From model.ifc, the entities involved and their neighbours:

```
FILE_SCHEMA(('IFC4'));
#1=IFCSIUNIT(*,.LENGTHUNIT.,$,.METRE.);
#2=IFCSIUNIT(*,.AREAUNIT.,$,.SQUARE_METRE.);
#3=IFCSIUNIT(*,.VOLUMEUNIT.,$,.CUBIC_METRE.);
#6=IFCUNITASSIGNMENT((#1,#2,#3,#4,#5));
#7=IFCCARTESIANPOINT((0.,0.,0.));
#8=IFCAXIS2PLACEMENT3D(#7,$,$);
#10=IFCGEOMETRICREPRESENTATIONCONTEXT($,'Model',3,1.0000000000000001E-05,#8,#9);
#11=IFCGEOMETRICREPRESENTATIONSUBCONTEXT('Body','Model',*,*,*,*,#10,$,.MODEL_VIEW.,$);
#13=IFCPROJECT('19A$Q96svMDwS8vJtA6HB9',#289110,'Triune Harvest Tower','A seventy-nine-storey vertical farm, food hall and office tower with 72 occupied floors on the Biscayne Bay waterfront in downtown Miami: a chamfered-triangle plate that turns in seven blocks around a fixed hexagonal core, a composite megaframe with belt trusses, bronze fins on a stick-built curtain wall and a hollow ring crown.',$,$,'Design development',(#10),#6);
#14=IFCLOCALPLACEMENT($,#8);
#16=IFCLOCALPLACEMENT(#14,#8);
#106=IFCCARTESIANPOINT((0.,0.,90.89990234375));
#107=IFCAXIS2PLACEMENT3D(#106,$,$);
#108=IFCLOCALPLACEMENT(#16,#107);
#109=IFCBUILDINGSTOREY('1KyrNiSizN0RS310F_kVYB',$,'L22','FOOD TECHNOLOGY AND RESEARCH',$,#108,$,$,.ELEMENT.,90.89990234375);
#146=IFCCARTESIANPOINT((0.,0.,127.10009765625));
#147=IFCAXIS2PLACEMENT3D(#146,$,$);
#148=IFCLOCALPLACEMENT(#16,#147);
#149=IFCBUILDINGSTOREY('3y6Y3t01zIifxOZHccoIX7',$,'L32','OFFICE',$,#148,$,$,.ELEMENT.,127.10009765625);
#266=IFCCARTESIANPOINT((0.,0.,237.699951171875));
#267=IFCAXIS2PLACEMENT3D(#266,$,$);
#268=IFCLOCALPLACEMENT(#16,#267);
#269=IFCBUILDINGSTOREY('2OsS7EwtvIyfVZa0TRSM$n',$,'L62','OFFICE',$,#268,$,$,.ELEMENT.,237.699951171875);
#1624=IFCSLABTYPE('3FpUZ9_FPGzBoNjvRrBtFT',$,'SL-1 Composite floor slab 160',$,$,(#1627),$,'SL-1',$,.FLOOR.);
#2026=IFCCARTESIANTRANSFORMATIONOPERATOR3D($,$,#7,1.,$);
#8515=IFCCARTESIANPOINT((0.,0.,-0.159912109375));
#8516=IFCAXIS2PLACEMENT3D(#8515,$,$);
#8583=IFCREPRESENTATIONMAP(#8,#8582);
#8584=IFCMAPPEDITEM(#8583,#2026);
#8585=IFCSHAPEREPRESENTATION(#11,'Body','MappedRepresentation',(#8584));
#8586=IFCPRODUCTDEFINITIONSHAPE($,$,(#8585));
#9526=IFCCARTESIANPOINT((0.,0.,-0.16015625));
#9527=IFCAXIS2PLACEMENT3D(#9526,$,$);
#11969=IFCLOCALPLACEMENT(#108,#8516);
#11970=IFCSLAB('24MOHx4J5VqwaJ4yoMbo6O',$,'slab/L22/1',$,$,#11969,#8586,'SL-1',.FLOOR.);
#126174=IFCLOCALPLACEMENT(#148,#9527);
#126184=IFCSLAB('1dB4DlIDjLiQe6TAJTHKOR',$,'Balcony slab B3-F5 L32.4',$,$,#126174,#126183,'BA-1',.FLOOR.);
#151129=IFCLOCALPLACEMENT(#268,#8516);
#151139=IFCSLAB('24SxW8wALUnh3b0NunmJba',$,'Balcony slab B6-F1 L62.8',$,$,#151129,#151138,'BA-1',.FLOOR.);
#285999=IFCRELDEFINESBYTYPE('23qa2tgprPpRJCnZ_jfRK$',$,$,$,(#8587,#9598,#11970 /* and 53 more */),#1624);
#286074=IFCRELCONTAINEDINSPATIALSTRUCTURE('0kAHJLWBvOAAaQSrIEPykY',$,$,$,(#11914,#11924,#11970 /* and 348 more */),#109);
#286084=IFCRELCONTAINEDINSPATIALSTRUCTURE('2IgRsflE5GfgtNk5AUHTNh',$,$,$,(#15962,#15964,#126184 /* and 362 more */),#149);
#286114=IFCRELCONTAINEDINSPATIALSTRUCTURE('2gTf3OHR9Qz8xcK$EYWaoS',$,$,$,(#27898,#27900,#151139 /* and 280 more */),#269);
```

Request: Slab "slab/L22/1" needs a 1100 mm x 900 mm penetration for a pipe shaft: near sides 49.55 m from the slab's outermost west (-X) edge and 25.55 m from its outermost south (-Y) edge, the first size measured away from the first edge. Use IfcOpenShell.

```python
import numpy as np
import ifcopenshell
import ifcopenshell.api.feature
import ifcopenshell.api.geometry
import ifcopenshell.api.root
import ifcopenshell.geom
import ifcopenshell.util.placement
import ifcopenshell.util.representation
import ifcopenshell.util.shape
import ifcopenshell.util.unit

model = ifcopenshell.open("model.ifc")
unit_scale = ifcopenshell.util.unit.calculate_unit_scale(model)
settings = ifcopenshell.geom.settings()


def volume(element):
    """Net volume in cubic metres, openings subtracted."""
    shape = ifcopenshell.geom.create_shape(settings, element)
    return ifcopenshell.util.shape.get_volume(shape.geometry)


slab = model.by_guid("24MOHx4J5VqwaJ4yoMbo6O")
before = volume(slab)

# Extent in the slab's own axes, in metres. The edges named are its -X and -Y sides.
slab_shape = ifcopenshell.geom.create_shape(settings, slab)
vertices = ifcopenshell.util.shape.get_vertices(slab_shape.geometry)
x_min, y_min, bottom = vertices.min(axis=0)
top = vertices[:, 2].max()

opening = ifcopenshell.api.root.create_entity(model, ifc_class="IfcOpeningElement", name="Pipe shaft opening", predefined_type="OPENING")
context = ifcopenshell.util.representation.get_context(model, "Model", "Body", "MODEL_VIEW")
width, depth = 1.1, 0.9
outline = [(0.0, 0.0), (width, 0.0), (width, depth), (0.0, depth), (0.0, 0.0)]
# Overshoot both faces by 50 mm so the cut is clean.
shape = ifcopenshell.api.geometry.add_slab_representation(
    model, context=context, depth=top - bottom + 0.1, polyline=outline
)
ifcopenshell.api.geometry.assign_representation(model, product=opening, representation=shape)

matrix = ifcopenshell.util.placement.get_local_placement(slab.ObjectPlacement)
matrix[:, 3] = matrix @ np.append(np.array([x_min + 49.55, y_min + 25.55, bottom - 0.05]) / unit_scale, 1.0)
ifcopenshell.api.geometry.edit_object_placement(model, product=opening, matrix=matrix, is_si=False)
ifcopenshell.api.feature.add_feature(model, feature=opening, element=slab)

after = volume(slab)

print(f"slab volume {before:.3f} -> {after:.3f} m3")

model.write("model-out.ifc")
```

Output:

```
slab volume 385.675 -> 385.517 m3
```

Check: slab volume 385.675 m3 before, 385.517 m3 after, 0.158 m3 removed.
